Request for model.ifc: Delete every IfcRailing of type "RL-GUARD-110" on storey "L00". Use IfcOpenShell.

First a look at what the model holds.

```python
import ifcopenshell
import ifcopenshell.util.element

model = ifcopenshell.open("model.ifc")
print(model.schema)
storey = next(s for s in model.by_type("IfcBuildingStorey") if s.Name == "L00")
railings = [e for e in ifcopenshell.util.element.get_decomposition(storey) if e.is_a("IfcRailing")]
seen = {}
for e in railings:
    element_type = ifcopenshell.util.element.get_type(e)
    name = element_type.Name if element_type not in (None, e) else None
    seen[name] = seen.get(name, 0) + 1
for name, count in sorted(seen.items(), key=str):
    print(count, "x", name)
```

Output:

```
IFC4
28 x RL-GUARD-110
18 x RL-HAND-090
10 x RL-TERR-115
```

```python
import ifcopenshell
import ifcopenshell.api.root
import ifcopenshell.util.element

model = ifcopenshell.open("model.ifc")

storey = next(s for s in model.by_type("IfcBuildingStorey") if s.Name == "L00")
railings = [e for e in ifcopenshell.util.element.get_decomposition(storey) if e.is_a("IfcRailing")]
targets = [e for e in railings if (t := ifcopenshell.util.element.get_type(e)) not in (None, e) and t.Name == "RL-GUARD-110"]

for e in targets:
    ifcopenshell.api.root.remove_product(model, product=e)
print(len(targets), "removed")

model.write("model_v2.ifc")
```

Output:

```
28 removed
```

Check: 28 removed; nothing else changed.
